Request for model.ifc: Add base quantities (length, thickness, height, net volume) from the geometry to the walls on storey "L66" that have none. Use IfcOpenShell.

First a look at what the model holds.

```python
import ifcopenshell
import ifcopenshell.util.element
import ifcopenshell.util.unit

model = ifcopenshell.open("model.ifc")
print(model.schema)
for unit_type in ("LENGTHUNIT", "AREAUNIT", "VOLUMEUNIT"):
    print(unit_type, ifcopenshell.util.unit.calculate_unit_scale(model, unit_type))
storey = next(s for s in model.by_type("IfcBuildingStorey") if s.Name == "L66")
walls = [e for e in ifcopenshell.util.element.get_decomposition(storey) if e.is_a("IfcWall")]
for e in sorted(walls, key=lambda e: e.id()):
    print(e.id(), e.is_a(), e.Name, list(ifcopenshell.util.element.get_psets(e, qtos_only=True)), sep=" | ")
```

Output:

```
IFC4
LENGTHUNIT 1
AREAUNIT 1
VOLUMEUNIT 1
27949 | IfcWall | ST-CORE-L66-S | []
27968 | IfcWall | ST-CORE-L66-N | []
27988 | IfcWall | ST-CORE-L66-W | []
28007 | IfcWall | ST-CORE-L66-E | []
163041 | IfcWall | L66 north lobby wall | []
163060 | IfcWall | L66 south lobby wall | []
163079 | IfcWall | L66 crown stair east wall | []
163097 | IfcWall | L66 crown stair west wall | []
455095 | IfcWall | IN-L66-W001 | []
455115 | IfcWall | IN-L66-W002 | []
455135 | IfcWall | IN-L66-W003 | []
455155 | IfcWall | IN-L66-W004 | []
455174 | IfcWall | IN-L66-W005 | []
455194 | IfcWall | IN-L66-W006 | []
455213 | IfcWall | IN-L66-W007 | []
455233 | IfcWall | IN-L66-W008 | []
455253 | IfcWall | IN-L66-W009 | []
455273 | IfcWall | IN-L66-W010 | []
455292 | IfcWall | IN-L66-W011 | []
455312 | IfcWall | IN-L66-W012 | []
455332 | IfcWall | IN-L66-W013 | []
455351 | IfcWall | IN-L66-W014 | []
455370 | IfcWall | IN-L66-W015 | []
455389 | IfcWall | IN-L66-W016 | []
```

```python
import ifcopenshell
import ifcopenshell.api.pset
import ifcopenshell.geom
import ifcopenshell.util.element
import ifcopenshell.util.shape
import ifcopenshell.util.unit

model = ifcopenshell.open("model.ifc")
unit_scale = ifcopenshell.util.unit.calculate_unit_scale(model)
volume_scale = ifcopenshell.util.unit.calculate_unit_scale(model, "VOLUMEUNIT")
settings = ifcopenshell.geom.settings()

storey = next(s for s in model.by_type("IfcBuildingStorey") if s.Name == "L66")
walls = [e for e in ifcopenshell.util.element.get_decomposition(storey) if e.is_a("IfcWall")]

for e in sorted(walls, key=lambda e: e.id()):
    if ifcopenshell.util.element.get_psets(e, qtos_only=True, should_inherit=False):
        continue
    # Geometry comes back in metres, in the element's own axes.
    shape = ifcopenshell.geom.create_shape(settings, e)
    values = {
        "Length": ifcopenshell.util.shape.get_x(shape.geometry) / unit_scale,
        "Width": ifcopenshell.util.shape.get_y(shape.geometry) / unit_scale,
        "Height": ifcopenshell.util.shape.get_z(shape.geometry) / unit_scale,
        "NetVolume": ifcopenshell.util.shape.get_volume(shape.geometry) / volume_scale,
    }
    qto = ifcopenshell.api.pset.add_qto(model, product=e, name="Qto_WallBaseQuantities")
    ifcopenshell.api.pset.edit_qto(model, qto=qto, properties=values)
    print(e.id(), {k: round(v, 3) for k, v in values.items()})

model.write("model_updated.ifc")
```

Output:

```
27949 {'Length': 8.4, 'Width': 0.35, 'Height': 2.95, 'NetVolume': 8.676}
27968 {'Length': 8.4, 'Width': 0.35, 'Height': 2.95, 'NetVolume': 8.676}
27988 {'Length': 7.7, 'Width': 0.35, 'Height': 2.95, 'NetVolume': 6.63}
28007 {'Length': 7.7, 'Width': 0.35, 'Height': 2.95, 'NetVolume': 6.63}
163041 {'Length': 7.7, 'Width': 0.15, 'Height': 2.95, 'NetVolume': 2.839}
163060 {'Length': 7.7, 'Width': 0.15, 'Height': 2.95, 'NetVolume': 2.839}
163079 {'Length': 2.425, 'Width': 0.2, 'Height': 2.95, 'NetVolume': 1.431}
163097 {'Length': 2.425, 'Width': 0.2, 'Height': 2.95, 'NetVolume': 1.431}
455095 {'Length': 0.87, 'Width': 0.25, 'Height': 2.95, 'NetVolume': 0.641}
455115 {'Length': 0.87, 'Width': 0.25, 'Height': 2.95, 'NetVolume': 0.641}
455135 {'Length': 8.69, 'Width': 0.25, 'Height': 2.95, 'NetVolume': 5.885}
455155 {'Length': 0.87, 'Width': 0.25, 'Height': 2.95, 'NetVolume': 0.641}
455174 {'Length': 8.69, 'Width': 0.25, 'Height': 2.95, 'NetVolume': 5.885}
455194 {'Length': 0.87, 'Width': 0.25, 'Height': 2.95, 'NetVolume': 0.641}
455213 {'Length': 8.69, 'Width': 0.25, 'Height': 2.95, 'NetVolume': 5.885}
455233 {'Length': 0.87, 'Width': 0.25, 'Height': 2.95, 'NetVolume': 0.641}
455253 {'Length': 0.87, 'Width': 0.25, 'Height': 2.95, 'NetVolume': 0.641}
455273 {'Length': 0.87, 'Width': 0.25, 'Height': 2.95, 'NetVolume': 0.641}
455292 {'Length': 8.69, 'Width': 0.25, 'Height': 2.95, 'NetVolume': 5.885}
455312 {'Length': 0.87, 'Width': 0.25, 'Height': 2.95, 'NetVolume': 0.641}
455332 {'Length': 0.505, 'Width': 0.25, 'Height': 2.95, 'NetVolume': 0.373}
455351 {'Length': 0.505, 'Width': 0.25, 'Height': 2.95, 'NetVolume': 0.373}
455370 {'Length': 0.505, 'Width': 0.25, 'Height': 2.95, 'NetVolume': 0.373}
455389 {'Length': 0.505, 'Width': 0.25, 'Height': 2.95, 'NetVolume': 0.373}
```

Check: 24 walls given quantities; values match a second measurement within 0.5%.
